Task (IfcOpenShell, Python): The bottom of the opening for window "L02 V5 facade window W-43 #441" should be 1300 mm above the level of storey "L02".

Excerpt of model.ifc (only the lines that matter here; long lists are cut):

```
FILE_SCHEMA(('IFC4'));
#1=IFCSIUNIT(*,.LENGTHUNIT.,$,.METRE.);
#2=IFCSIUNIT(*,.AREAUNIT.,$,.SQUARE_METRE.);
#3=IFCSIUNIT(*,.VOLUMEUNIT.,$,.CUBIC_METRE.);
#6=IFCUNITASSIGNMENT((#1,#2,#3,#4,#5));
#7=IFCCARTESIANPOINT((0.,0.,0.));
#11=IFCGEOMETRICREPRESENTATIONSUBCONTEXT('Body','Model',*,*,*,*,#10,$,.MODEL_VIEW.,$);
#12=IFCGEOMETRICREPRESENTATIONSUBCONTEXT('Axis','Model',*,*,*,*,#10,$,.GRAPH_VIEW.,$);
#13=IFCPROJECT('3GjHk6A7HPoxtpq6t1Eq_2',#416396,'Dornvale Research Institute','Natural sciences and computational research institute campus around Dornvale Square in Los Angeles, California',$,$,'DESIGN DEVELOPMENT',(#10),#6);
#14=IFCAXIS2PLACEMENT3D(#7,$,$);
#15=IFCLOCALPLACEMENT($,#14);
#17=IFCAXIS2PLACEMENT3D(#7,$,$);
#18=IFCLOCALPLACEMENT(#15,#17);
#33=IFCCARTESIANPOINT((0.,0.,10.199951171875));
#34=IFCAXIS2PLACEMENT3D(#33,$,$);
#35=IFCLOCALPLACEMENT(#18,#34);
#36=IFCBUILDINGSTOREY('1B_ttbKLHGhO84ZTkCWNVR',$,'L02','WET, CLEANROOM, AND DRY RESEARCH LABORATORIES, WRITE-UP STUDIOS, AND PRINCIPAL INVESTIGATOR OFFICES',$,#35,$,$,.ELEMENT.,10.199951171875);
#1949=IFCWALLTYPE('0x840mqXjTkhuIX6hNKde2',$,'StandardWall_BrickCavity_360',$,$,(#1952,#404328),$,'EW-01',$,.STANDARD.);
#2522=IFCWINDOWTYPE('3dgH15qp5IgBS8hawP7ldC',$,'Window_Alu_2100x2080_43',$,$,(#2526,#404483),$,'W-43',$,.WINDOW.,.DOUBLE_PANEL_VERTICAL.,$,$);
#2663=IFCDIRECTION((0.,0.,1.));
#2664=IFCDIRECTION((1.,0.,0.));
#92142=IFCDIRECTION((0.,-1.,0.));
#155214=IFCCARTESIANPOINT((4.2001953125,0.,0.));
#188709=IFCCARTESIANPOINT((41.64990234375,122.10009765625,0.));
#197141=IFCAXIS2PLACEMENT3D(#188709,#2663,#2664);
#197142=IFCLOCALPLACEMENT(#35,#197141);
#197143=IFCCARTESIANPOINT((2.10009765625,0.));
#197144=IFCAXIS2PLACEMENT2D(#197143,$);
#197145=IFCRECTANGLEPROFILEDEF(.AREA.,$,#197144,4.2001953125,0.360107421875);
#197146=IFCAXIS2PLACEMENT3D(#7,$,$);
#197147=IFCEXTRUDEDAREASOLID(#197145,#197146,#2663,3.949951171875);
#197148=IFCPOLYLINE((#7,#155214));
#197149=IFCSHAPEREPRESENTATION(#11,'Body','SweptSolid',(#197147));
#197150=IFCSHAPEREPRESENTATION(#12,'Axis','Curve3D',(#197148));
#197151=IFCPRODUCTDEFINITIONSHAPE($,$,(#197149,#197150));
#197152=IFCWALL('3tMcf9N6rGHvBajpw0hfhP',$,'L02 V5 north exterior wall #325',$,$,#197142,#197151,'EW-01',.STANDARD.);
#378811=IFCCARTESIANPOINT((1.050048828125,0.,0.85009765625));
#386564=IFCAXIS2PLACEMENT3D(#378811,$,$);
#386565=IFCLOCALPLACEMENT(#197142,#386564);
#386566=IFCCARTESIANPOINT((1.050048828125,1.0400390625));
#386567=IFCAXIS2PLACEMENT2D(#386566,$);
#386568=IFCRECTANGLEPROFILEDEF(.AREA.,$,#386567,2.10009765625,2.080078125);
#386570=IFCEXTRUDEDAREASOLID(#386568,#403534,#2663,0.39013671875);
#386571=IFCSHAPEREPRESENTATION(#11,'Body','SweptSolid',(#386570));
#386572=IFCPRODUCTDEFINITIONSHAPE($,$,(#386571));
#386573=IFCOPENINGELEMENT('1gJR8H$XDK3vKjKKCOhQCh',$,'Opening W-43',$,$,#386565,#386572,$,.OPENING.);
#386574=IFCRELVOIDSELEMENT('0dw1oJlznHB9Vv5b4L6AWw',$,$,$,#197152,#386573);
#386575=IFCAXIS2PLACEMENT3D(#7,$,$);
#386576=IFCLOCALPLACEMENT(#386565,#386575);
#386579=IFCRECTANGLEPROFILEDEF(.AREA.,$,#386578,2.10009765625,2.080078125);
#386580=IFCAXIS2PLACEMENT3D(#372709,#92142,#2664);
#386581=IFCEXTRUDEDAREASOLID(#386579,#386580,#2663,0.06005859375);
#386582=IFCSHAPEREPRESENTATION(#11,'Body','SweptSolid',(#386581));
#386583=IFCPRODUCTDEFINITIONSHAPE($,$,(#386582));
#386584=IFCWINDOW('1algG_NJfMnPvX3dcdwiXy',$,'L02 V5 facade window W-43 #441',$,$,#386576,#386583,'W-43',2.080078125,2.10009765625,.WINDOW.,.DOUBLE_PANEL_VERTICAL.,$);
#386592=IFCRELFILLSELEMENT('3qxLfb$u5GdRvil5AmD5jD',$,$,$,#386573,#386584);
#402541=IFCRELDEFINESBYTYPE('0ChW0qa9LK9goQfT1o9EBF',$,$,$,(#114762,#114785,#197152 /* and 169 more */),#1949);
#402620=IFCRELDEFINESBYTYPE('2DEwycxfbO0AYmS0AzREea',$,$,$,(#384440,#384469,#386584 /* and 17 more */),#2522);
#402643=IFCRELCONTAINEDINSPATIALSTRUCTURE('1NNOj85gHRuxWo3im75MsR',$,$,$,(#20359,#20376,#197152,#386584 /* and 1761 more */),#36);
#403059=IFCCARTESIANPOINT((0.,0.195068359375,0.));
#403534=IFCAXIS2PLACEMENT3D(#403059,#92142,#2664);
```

```python
import numpy as np
import ifcopenshell
import ifcopenshell.api.geometry
import ifcopenshell.geom
import ifcopenshell.util.element
import ifcopenshell.util.placement
import ifcopenshell.util.shape
import ifcopenshell.util.unit

model = ifcopenshell.open("model.ifc")
unit_scale = ifcopenshell.util.unit.calculate_unit_scale(model)

window = model.by_guid("1algG_NJfMnPvX3dcdwiXy")
opening = window.FillsVoids[0].RelatingOpeningElement
storey = ifcopenshell.util.element.get_container(window, ifc_class="IfcBuildingStorey")
level = ifcopenshell.util.placement.get_local_placement(storey.ObjectPlacement)[2, 3]

# The opening's origin need not be at the sill, so measure its lowest point.
shape = ifcopenshell.geom.create_shape(ifcopenshell.geom.settings(), opening)
bottom = ifcopenshell.util.shape.get_shape_bottom_elevation(shape, shape.geometry) / unit_scale
dz = level + 1.3 - bottom

shift = np.array([0.0, 0.0, dz])
# The window is placed relative to its opening, so it follows when the opening moves.
matrix = ifcopenshell.util.placement.get_local_placement(opening.ObjectPlacement)
matrix[:3, 3] += shift
ifcopenshell.api.geometry.edit_object_placement(
    model, product=opening, matrix=matrix, is_si=False, should_transform_children=True
)

print(f"moved by {dz * unit_scale:+.3f} m")

model.write("model_updated.ifc")
```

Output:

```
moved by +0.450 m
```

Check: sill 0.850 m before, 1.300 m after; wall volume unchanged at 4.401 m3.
